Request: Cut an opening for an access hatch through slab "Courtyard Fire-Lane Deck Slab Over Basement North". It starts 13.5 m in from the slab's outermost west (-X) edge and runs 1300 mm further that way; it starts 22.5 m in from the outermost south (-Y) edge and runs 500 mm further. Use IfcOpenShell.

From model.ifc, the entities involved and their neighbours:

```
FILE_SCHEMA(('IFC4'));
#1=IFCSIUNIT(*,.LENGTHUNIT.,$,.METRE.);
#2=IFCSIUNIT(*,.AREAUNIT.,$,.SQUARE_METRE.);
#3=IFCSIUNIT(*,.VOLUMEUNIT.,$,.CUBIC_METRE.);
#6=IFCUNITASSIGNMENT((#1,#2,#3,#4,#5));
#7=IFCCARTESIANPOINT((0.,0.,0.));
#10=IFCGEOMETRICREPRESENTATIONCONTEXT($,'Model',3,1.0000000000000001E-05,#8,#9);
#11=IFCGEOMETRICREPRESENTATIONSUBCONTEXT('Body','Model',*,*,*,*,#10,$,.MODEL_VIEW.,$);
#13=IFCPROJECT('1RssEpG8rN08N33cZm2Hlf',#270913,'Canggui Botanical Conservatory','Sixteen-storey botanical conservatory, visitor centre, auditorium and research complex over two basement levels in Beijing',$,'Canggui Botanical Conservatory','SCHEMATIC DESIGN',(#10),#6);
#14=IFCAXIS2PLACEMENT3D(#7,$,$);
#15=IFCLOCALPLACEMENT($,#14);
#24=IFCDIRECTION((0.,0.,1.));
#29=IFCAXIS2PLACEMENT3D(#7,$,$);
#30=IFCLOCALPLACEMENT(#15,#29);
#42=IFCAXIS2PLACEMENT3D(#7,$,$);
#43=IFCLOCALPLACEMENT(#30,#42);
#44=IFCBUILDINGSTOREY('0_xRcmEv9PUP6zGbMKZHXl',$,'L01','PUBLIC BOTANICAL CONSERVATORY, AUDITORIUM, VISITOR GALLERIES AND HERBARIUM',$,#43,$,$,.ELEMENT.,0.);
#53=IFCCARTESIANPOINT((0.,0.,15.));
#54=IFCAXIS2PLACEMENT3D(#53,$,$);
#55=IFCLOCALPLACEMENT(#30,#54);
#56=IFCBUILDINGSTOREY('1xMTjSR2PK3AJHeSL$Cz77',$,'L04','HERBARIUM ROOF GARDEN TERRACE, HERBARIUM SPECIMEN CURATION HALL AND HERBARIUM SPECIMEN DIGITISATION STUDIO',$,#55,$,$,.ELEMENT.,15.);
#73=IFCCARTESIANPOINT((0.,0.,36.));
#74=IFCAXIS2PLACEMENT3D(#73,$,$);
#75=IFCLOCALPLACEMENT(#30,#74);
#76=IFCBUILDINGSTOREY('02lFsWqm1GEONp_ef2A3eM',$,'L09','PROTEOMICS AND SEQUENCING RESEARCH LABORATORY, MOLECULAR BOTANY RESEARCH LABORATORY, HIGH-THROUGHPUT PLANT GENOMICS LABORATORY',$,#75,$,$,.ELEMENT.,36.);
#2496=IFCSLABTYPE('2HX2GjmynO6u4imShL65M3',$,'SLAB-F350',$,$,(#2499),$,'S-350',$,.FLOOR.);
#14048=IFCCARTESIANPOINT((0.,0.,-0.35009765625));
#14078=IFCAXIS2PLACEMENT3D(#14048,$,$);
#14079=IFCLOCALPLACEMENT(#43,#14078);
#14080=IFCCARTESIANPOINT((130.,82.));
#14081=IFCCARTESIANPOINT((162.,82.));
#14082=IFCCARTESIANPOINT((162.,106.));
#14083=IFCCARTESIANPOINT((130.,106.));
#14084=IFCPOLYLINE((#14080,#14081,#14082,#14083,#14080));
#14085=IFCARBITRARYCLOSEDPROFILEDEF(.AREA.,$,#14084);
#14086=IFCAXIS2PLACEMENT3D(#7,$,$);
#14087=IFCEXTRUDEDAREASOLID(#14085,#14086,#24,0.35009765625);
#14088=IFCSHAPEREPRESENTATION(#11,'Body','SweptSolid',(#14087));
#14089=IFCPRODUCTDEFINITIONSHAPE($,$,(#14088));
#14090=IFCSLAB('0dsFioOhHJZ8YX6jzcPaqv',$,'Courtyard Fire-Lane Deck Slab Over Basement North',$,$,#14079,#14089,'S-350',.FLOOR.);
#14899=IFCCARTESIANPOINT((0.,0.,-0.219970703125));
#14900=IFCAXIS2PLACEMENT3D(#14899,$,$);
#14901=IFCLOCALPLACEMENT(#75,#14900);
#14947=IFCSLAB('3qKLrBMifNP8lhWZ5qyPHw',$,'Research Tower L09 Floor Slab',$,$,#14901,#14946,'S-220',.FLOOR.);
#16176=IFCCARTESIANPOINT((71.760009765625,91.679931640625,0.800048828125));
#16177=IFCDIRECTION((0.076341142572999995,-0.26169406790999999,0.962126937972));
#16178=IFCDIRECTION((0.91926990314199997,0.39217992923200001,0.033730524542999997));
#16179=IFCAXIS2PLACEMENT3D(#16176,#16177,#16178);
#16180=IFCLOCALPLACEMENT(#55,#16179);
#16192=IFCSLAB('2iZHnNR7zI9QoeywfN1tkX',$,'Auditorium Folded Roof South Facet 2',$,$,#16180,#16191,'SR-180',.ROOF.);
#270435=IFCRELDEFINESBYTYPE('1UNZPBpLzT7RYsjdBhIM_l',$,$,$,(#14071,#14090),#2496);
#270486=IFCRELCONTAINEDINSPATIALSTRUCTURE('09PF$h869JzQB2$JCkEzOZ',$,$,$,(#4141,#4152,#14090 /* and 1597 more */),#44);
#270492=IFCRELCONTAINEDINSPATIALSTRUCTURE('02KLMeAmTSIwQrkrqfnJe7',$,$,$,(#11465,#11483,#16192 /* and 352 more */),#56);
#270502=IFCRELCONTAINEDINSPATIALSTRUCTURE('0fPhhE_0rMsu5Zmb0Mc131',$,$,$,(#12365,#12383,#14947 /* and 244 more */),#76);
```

```python
import numpy as np
import ifcopenshell
import ifcopenshell.api.feature
import ifcopenshell.api.geometry
import ifcopenshell.api.root
import ifcopenshell.geom
import ifcopenshell.util.placement
import ifcopenshell.util.representation
import ifcopenshell.util.shape
import ifcopenshell.util.unit

model = ifcopenshell.open("model.ifc")
unit_scale = ifcopenshell.util.unit.calculate_unit_scale(model)
settings = ifcopenshell.geom.settings()


def volume(element):
    """Net volume in cubic metres, openings subtracted."""
    shape = ifcopenshell.geom.create_shape(settings, element)
    return ifcopenshell.util.shape.get_volume(shape.geometry)


slab = model.by_guid("0dsFioOhHJZ8YX6jzcPaqv")
before = volume(slab)

# Extent in the slab's own axes, in metres. The edges named are its -X and -Y sides.
slab_shape = ifcopenshell.geom.create_shape(settings, slab)
vertices = ifcopenshell.util.shape.get_vertices(slab_shape.geometry)
x_min, y_min, bottom = vertices.min(axis=0)
top = vertices[:, 2].max()

opening = ifcopenshell.api.root.create_entity(model, ifc_class="IfcOpeningElement", name="Access hatch opening", predefined_type="OPENING")
context = ifcopenshell.util.representation.get_context(model, "Model", "Body", "MODEL_VIEW")
width, depth = 1.3, 0.5
outline = [(0.0, 0.0), (width, 0.0), (width, depth), (0.0, depth), (0.0, 0.0)]
# Overshoot both faces by 50 mm so the cut is clean.
shape = ifcopenshell.api.geometry.add_slab_representation(
    model, context=context, depth=top - bottom + 0.1, polyline=outline
)
ifcopenshell.api.geometry.assign_representation(model, product=opening, representation=shape)

matrix = ifcopenshell.util.placement.get_local_placement(slab.ObjectPlacement)
matrix[:, 3] = matrix @ np.append(np.array([x_min + 13.5, y_min + 22.5, bottom - 0.05]) / unit_scale, 1.0)
ifcopenshell.api.geometry.edit_object_placement(model, product=opening, matrix=matrix, is_si=False)
ifcopenshell.api.feature.add_feature(model, feature=opening, element=slab)

after = volume(slab)

print(f"slab volume {before:.3f} -> {after:.3f} m3")

model.write("model_v2.ifc")
```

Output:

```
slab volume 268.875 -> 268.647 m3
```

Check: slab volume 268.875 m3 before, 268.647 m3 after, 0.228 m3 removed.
